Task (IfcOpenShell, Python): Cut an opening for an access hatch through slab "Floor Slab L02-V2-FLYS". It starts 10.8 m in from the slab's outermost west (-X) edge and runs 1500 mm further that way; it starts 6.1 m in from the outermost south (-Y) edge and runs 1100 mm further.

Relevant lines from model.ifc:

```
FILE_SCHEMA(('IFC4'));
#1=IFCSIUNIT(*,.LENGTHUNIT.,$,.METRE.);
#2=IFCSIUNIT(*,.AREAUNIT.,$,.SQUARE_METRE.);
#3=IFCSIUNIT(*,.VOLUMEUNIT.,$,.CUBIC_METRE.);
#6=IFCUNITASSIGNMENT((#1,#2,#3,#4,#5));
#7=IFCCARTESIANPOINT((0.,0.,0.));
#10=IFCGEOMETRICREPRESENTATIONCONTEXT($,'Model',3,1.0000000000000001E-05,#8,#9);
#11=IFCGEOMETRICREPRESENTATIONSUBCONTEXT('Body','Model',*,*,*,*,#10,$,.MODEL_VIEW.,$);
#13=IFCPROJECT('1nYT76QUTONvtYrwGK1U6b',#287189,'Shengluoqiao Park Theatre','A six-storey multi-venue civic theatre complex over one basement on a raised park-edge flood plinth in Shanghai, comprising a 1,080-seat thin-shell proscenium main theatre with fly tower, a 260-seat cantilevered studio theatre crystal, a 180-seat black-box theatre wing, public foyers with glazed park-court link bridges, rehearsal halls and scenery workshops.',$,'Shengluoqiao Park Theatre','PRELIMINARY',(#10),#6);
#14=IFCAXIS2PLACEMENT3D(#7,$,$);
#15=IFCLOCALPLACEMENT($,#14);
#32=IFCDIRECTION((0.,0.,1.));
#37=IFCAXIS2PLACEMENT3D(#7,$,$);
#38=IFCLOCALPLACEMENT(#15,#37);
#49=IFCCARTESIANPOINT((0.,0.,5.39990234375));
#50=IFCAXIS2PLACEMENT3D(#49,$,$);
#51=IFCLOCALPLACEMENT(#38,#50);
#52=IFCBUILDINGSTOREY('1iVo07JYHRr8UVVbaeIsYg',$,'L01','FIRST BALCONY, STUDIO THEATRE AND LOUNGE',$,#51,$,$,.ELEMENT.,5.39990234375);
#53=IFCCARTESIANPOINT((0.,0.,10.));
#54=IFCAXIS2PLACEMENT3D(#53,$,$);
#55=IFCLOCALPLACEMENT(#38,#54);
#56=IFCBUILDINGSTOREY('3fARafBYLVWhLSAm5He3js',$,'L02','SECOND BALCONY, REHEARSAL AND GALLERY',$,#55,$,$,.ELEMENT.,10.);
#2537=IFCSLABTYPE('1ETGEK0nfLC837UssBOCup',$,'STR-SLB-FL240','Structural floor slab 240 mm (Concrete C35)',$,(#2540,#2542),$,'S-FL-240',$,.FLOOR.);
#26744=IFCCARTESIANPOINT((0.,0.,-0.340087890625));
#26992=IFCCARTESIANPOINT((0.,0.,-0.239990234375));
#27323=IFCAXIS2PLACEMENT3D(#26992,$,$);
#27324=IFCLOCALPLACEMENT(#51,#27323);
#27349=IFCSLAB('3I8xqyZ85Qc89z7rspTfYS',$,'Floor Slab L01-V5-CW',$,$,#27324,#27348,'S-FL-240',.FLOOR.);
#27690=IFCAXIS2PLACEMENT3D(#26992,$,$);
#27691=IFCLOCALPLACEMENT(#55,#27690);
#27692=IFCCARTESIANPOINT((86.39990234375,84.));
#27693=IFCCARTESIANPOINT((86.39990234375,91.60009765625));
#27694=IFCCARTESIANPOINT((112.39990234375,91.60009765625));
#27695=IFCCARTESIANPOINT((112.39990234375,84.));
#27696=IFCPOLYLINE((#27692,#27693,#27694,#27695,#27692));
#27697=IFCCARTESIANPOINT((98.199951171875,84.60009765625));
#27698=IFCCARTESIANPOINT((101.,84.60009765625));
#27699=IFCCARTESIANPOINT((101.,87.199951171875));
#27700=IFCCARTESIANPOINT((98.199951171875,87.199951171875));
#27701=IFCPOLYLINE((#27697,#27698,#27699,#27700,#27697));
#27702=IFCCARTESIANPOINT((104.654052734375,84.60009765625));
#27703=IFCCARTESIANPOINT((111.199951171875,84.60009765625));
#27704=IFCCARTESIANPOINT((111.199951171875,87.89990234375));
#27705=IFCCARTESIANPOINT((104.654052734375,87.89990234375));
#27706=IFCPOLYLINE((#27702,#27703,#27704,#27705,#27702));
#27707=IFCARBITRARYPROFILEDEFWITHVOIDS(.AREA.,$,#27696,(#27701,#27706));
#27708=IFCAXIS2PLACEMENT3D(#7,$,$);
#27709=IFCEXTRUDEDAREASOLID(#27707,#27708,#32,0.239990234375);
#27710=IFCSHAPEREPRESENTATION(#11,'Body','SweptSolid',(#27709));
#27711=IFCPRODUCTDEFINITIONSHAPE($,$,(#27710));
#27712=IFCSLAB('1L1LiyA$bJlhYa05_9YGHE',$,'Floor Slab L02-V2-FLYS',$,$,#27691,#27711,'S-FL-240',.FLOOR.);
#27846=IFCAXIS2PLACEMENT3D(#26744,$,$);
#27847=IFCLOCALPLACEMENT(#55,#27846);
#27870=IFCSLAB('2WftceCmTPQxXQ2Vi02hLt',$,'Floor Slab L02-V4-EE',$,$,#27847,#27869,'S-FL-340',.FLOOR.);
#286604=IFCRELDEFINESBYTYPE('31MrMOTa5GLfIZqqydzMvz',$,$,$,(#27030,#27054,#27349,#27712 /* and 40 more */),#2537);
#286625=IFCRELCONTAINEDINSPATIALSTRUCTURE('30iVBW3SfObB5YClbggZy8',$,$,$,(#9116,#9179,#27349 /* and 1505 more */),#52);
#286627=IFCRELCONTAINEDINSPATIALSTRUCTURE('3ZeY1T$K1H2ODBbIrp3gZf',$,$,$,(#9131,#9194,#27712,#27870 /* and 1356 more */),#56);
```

```python
import numpy as np
import ifcopenshell
import ifcopenshell.api.feature
import ifcopenshell.api.geometry
import ifcopenshell.api.root
import ifcopenshell.geom
import ifcopenshell.util.placement
import ifcopenshell.util.representation
import ifcopenshell.util.shape
import ifcopenshell.util.unit

model = ifcopenshell.open("model.ifc")
unit_scale = ifcopenshell.util.unit.calculate_unit_scale(model)
settings = ifcopenshell.geom.settings()


def volume(element):
    """Net volume in cubic metres, openings subtracted."""
    shape = ifcopenshell.geom.create_shape(settings, element)
    return ifcopenshell.util.shape.get_volume(shape.geometry)


slab = model.by_id(27712)
before = volume(slab)

# Extent in the slab's own axes, in metres. The edges named are its -X and -Y sides.
slab_shape = ifcopenshell.geom.create_shape(settings, slab)
vertices = ifcopenshell.util.shape.get_vertices(slab_shape.geometry)
x_min, y_min, bottom = vertices.min(axis=0)
top = vertices[:, 2].max()

opening = ifcopenshell.api.root.create_entity(model, ifc_class="IfcOpeningElement", name="Access hatch opening", predefined_type="OPENING")
context = ifcopenshell.util.representation.get_context(model, "Model", "Body", "MODEL_VIEW")
width, depth = 1.5, 1.1
outline = [(0.0, 0.0), (width, 0.0), (width, depth), (0.0, depth), (0.0, 0.0)]
# Overshoot both faces by 50 mm so the cut is clean.
shape = ifcopenshell.api.geometry.add_slab_representation(
    model, context=context, depth=top - bottom + 0.1, polyline=outline
)
ifcopenshell.api.geometry.assign_representation(model, product=opening, representation=shape)

matrix = ifcopenshell.util.placement.get_local_placement(slab.ObjectPlacement)
matrix[:, 3] = matrix @ np.append(np.array([x_min + 10.8, y_min + 6.1, bottom - 0.05]) / unit_scale, 1.0)
ifcopenshell.api.geometry.edit_object_placement(model, product=opening, matrix=matrix, is_si=False)
ifcopenshell.api.feature.add_feature(model, feature=opening, element=slab)

after = volume(slab)

print(f"slab volume {before:.3f} -> {after:.3f} m3")

model.write("model_rev.ifc")
```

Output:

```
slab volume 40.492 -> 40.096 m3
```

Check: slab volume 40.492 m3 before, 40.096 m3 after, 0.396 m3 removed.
